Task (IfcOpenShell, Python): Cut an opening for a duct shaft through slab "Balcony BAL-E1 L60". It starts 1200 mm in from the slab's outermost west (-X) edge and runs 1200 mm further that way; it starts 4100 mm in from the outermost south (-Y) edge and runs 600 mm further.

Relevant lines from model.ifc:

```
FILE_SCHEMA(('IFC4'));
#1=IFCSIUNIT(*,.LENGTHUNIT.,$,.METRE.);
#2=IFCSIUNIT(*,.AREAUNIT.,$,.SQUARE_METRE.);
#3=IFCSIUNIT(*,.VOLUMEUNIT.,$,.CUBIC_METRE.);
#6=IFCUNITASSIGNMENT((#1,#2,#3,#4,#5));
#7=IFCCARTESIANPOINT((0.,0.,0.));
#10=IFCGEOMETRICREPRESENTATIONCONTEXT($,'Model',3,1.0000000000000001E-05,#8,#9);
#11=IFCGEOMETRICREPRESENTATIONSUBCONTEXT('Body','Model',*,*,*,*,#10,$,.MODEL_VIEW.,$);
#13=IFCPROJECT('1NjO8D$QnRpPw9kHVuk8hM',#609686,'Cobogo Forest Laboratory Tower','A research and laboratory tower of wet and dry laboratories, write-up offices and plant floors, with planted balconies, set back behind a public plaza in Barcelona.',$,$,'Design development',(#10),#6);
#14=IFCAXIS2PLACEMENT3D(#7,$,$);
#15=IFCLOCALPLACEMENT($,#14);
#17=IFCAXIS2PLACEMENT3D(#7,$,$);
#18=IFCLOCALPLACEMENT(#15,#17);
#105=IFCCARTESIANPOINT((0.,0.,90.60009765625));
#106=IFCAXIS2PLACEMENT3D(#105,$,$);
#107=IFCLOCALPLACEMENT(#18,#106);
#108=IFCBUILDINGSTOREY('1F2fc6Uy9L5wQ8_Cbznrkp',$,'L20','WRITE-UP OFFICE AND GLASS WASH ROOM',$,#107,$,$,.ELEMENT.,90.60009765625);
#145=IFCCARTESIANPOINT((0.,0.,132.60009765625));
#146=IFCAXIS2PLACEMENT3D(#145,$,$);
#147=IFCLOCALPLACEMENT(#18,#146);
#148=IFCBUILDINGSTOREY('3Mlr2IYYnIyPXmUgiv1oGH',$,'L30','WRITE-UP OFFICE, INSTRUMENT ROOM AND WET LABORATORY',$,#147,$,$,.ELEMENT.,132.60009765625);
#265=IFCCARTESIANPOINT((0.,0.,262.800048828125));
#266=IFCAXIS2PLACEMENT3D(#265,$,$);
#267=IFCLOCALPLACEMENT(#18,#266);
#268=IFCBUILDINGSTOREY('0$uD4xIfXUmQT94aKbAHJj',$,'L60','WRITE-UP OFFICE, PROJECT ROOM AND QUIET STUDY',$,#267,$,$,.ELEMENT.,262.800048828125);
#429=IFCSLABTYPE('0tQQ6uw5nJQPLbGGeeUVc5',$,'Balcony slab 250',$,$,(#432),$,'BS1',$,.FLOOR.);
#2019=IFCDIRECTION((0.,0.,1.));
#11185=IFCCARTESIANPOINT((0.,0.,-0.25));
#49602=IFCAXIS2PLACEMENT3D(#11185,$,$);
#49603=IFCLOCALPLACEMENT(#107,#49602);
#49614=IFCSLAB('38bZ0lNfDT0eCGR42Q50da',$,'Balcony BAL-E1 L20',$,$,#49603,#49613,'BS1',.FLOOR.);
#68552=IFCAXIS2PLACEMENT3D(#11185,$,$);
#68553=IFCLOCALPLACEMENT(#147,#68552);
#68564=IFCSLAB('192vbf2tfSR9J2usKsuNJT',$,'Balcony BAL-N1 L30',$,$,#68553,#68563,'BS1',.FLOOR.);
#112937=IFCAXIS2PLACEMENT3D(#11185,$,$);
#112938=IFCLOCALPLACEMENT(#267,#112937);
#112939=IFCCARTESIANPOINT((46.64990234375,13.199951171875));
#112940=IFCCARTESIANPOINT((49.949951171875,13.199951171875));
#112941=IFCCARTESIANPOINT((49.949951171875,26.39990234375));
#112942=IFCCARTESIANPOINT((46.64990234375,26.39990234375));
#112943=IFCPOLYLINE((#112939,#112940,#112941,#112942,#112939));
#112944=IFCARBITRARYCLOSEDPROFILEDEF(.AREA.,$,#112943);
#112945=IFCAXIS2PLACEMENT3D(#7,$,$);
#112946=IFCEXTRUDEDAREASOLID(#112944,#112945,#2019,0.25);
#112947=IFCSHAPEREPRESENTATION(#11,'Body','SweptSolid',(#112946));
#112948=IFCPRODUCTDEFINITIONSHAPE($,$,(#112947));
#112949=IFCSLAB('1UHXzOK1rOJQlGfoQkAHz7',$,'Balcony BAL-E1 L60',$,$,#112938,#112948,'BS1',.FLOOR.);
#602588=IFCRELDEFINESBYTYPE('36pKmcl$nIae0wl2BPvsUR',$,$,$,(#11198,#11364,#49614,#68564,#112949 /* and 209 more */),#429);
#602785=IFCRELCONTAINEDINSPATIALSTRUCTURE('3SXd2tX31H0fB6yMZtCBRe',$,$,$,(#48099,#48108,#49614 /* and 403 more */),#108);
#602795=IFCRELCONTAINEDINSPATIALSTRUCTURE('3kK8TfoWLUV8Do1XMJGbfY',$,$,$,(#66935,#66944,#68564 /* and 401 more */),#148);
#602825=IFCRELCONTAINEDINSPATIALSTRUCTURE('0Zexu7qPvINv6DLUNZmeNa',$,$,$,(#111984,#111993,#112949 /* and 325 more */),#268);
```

```python
import numpy as np
import ifcopenshell
import ifcopenshell.api.feature
import ifcopenshell.api.geometry
import ifcopenshell.api.root
import ifcopenshell.geom
import ifcopenshell.util.placement
import ifcopenshell.util.representation
import ifcopenshell.util.shape
import ifcopenshell.util.unit

model = ifcopenshell.open("model.ifc")
unit_scale = ifcopenshell.util.unit.calculate_unit_scale(model)
settings = ifcopenshell.geom.settings()


def volume(element):
    """Net volume in cubic metres, openings subtracted."""
    shape = ifcopenshell.geom.create_shape(settings, element)
    return ifcopenshell.util.shape.get_volume(shape.geometry)


slab = model.by_guid("1UHXzOK1rOJQlGfoQkAHz7")
before = volume(slab)

# Extent in the slab's own axes, in metres. The edges named are its -X and -Y sides.
slab_shape = ifcopenshell.geom.create_shape(settings, slab)
vertices = ifcopenshell.util.shape.get_vertices(slab_shape.geometry)
x_min, y_min, bottom = vertices.min(axis=0)
top = vertices[:, 2].max()

opening = ifcopenshell.api.root.create_entity(model, ifc_class="IfcOpeningElement", name="Duct shaft opening", predefined_type="OPENING")
context = ifcopenshell.util.representation.get_context(model, "Model", "Body", "MODEL_VIEW")
width, depth = 1.2, 0.6
outline = [(0.0, 0.0), (width, 0.0), (width, depth), (0.0, depth), (0.0, 0.0)]
# Overshoot both faces by 50 mm so the cut is clean.
shape = ifcopenshell.api.geometry.add_slab_representation(
    model, context=context, depth=top - bottom + 0.1, polyline=outline
)
ifcopenshell.api.geometry.assign_representation(model, product=opening, representation=shape)

matrix = ifcopenshell.util.placement.get_local_placement(slab.ObjectPlacement)
matrix[:, 3] = matrix @ np.append(np.array([x_min + 1.2, y_min + 4.1, bottom - 0.05]) / unit_scale, 1.0)
ifcopenshell.api.geometry.edit_object_placement(model, product=opening, matrix=matrix, is_si=False)
ifcopenshell.api.feature.add_feature(model, feature=opening, element=slab)

after = volume(slab)

print(f"slab volume {before:.3f} -> {after:.3f} m3")

model.write("model_edited.ifc")
```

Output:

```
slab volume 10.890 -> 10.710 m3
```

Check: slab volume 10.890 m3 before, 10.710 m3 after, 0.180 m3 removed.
